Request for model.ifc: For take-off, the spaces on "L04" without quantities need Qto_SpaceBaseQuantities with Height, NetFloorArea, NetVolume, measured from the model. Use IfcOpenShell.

First a look at what the model holds.

```python
import ifcopenshell
import ifcopenshell.util.element
import ifcopenshell.util.unit

model = ifcopenshell.open("model.ifc")
print(model.schema)
for unit_type in ("LENGTHUNIT", "AREAUNIT", "VOLUMEUNIT"):
    print(unit_type, ifcopenshell.util.unit.calculate_unit_scale(model, unit_type))
storey = next(s for s in model.by_type("IfcBuildingStorey") if s.Name == "L04")
spaces = [e for e in ifcopenshell.util.element.get_decomposition(storey) if e.is_a("IfcSpace")]
for e in sorted(spaces, key=lambda e: e.id()):
    print(e.id(), e.is_a(), e.Name, list(ifcopenshell.util.element.get_psets(e, qtos_only=True)), sep=" | ")
```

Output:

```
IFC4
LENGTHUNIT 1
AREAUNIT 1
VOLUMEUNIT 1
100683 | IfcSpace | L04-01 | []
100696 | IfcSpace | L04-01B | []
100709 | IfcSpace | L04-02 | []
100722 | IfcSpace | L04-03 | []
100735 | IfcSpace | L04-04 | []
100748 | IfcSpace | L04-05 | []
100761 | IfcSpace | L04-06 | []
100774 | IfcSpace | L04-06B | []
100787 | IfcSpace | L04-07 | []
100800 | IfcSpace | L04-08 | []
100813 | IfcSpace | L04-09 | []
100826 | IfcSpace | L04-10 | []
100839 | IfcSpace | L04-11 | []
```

```python
import ifcopenshell
import ifcopenshell.api.pset
import ifcopenshell.geom
import ifcopenshell.util.element
import ifcopenshell.util.shape
import ifcopenshell.util.unit

model = ifcopenshell.open("model.ifc")
unit_scale = ifcopenshell.util.unit.calculate_unit_scale(model)
area_scale = ifcopenshell.util.unit.calculate_unit_scale(model, "AREAUNIT")
volume_scale = ifcopenshell.util.unit.calculate_unit_scale(model, "VOLUMEUNIT")
settings = ifcopenshell.geom.settings()

storey = next(s for s in model.by_type("IfcBuildingStorey") if s.Name == "L04")
spaces = [e for e in ifcopenshell.util.element.get_decomposition(storey) if e.is_a("IfcSpace")]

for e in sorted(spaces, key=lambda e: e.id()):
    if ifcopenshell.util.element.get_psets(e, qtos_only=True, should_inherit=False):
        continue
    # Geometry comes back in metres, in the element's own axes.
    shape = ifcopenshell.geom.create_shape(settings, e)
    values = {
        "Height": ifcopenshell.util.shape.get_z(shape.geometry) / unit_scale,
        "NetFloorArea": ifcopenshell.util.shape.get_footprint_area(shape.geometry) / area_scale,
        "NetVolume": ifcopenshell.util.shape.get_volume(shape.geometry) / volume_scale,
    }
    qto = ifcopenshell.api.pset.add_qto(model, product=e, name="Qto_SpaceBaseQuantities")
    ifcopenshell.api.pset.edit_qto(model, qto=qto, properties=values)
    print(e.id(), {k: round(v, 3) for k, v in values.items()})

model.write("model_edited.ifc")
```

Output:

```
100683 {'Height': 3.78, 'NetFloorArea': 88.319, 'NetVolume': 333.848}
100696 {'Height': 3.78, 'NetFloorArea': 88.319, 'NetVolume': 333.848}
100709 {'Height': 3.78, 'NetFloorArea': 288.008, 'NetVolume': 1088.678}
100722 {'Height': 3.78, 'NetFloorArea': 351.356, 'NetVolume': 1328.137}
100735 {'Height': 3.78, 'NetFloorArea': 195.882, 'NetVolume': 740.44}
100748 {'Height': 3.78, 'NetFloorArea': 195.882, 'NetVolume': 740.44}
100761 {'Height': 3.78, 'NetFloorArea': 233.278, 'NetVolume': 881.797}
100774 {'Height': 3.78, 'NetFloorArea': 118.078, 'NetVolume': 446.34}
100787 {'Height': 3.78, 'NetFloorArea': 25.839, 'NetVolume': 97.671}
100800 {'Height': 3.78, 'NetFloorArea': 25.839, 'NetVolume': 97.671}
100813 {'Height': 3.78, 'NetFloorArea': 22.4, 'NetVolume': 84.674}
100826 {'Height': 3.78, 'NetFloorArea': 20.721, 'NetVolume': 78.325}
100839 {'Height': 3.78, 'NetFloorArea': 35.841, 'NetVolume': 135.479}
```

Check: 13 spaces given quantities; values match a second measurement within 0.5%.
